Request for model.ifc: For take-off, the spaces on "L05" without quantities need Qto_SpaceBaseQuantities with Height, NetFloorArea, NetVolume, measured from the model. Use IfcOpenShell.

First a look at what the model holds.

```python
import ifcopenshell
import ifcopenshell.util.element
import ifcopenshell.util.unit

model = ifcopenshell.open("model.ifc")
print(model.schema)
for unit_type in ("LENGTHUNIT", "AREAUNIT", "VOLUMEUNIT"):
    print(unit_type, ifcopenshell.util.unit.calculate_unit_scale(model, unit_type))
storey = next(s for s in model.by_type("IfcBuildingStorey") if s.Name == "L05")
spaces = [e for e in ifcopenshell.util.element.get_decomposition(storey) if e.is_a("IfcSpace")]
for e in sorted(spaces, key=lambda e: e.id()):
    print(e.id(), e.is_a(), e.Name, list(ifcopenshell.util.element.get_psets(e, qtos_only=True)), sep=" | ")
```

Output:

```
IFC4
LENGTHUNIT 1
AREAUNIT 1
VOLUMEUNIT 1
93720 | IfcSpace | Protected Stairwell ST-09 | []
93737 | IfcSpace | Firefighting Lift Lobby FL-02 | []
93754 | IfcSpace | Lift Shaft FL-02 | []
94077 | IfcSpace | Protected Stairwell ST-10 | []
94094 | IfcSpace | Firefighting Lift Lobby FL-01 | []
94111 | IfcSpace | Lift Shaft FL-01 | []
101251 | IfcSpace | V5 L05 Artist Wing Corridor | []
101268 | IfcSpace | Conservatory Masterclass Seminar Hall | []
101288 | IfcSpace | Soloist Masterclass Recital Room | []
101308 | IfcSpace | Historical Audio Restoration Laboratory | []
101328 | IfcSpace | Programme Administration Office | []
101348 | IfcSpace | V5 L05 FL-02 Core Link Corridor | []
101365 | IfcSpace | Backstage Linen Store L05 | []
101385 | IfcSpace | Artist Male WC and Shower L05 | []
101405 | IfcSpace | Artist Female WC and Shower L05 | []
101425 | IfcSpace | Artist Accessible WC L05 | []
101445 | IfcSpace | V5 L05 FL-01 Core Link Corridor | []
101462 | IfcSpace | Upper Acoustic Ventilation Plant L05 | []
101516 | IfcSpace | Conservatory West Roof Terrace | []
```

```python
import ifcopenshell
import ifcopenshell.api.pset
import ifcopenshell.geom
import ifcopenshell.util.element
import ifcopenshell.util.shape
import ifcopenshell.util.unit

model = ifcopenshell.open("model.ifc")
unit_scale = ifcopenshell.util.unit.calculate_unit_scale(model)
area_scale = ifcopenshell.util.unit.calculate_unit_scale(model, "AREAUNIT")
volume_scale = ifcopenshell.util.unit.calculate_unit_scale(model, "VOLUMEUNIT")
settings = ifcopenshell.geom.settings()

storey = next(s for s in model.by_type("IfcBuildingStorey") if s.Name == "L05")
spaces = [e for e in ifcopenshell.util.element.get_decomposition(storey) if e.is_a("IfcSpace")]

for e in sorted(spaces, key=lambda e: e.id()):
    if ifcopenshell.util.element.get_psets(e, qtos_only=True, should_inherit=False):
        continue
    # Geometry comes back in metres, in the element's own axes.
    shape = ifcopenshell.geom.create_shape(settings, e)
    values = {
        "Height": ifcopenshell.util.shape.get_z(shape.geometry) / unit_scale,
        "NetFloorArea": ifcopenshell.util.shape.get_footprint_area(shape.geometry) / area_scale,
        "NetVolume": ifcopenshell.util.shape.get_volume(shape.geometry) / volume_scale,
    }
    qto = ifcopenshell.api.pset.add_qto(model, product=e, name="Qto_SpaceBaseQuantities")
    ifcopenshell.api.pset.edit_qto(model, qto=qto, properties=values)
    print(e.id(), {k: round(v, 3) for k, v in values.items()})

model.write("model_updated.ifc")
```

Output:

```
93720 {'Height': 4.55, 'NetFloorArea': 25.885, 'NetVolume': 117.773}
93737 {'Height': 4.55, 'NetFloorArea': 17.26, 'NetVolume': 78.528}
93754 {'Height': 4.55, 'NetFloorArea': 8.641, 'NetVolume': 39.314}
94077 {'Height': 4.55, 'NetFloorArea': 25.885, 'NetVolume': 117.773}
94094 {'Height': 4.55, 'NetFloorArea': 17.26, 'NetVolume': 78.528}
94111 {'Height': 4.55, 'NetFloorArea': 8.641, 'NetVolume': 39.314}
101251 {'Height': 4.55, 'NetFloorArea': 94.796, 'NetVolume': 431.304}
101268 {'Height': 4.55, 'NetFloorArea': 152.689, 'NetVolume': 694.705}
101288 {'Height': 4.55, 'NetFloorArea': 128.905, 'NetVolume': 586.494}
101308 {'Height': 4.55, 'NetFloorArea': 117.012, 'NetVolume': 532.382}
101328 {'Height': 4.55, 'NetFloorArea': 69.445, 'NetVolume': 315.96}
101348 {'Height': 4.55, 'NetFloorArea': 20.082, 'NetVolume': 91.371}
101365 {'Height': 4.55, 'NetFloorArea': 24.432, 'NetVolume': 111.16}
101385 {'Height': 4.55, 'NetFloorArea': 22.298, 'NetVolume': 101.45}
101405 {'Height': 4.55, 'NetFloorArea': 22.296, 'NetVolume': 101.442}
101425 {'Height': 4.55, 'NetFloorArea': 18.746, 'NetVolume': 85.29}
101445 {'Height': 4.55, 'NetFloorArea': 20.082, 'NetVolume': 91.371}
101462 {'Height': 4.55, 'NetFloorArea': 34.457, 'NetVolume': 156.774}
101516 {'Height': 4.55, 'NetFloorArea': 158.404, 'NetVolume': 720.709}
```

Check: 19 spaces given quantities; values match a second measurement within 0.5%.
